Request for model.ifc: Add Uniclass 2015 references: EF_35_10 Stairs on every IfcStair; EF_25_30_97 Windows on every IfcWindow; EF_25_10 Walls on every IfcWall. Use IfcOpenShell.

First a look at what the model holds.

```python
import ifcopenshell

model = ifcopenshell.open("model.ifc")
print(model.schema)
print("classifications:", [c.Name for c in model.by_type("IfcClassification")])
for ifc_class in ("IfcDoor", "IfcRoof", "IfcStair", "IfcWall", "IfcWindow"):
    print(ifc_class, len(model.by_type(ifc_class)))
```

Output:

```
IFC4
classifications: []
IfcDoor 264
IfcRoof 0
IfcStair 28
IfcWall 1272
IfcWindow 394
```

```python
import ifcopenshell
import ifcopenshell.api.classification

model = ifcopenshell.open("model.ifc")

system = ifcopenshell.api.classification.add_classification(model, classification="Uniclass 2015")

codes = {
    "IfcStair": ("EF_35_10", "Stairs"),
    "IfcWindow": ("EF_25_30_97", "Windows"),
    "IfcWall": ("EF_25_10", "Walls"),
}
for ifc_class, (code, name) in codes.items():
    products = model.by_type(ifc_class)
    ifcopenshell.api.classification.add_reference(
        model, products=products, classification=system, identification=code, name=name
    )
    print(code, len(products))

model.write("model_v2.ifc")
```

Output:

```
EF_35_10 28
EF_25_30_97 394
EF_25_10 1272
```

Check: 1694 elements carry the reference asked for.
